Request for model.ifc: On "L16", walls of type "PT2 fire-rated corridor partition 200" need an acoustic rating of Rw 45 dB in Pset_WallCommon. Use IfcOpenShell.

First a look at what the model holds.

```python
import ifcopenshell
import ifcopenshell.util.element

model = ifcopenshell.open("model.ifc")
print(model.schema)
storey = next(s for s in model.by_type("IfcBuildingStorey") if s.Name == "L16")
walls = [e for e in ifcopenshell.util.element.get_decomposition(storey) if e.is_a("IfcWall")]
seen = {}
for e in walls:
    element_type = ifcopenshell.util.element.get_type(e)
    key = (element_type.Name if element_type != e and element_type else None, ifcopenshell.util.element.get_pset(e, "Pset_WallCommon", "AcousticRating"))
    seen[key] = seen.get(key, 0) + 1
for (name, value), count in sorted(seen.items(), key=str):
    print(count, "x", name, "|", value)
```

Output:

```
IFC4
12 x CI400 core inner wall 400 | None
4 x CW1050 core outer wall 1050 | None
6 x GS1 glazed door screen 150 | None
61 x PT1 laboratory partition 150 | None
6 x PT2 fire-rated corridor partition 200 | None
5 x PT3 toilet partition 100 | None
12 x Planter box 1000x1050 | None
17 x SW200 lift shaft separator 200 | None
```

```python
import ifcopenshell
import ifcopenshell.api.pset
import ifcopenshell.util.element

model = ifcopenshell.open("model.ifc")

storey = next(s for s in model.by_type("IfcBuildingStorey") if s.Name == "L16")
walls = [e for e in ifcopenshell.util.element.get_decomposition(storey) if e.is_a("IfcWall")]

count = 0
for e in walls:
    element_type = ifcopenshell.util.element.get_type(e)
    if element_type in (None, e) or element_type.Name != "PT2 fire-rated corridor partition 200":
        continue
    found = ifcopenshell.util.element.get_pset(e, "Pset_WallCommon", should_inherit=False)
    if found:
        pset = model.by_id(found["id"])
        if len(ifcopenshell.util.element.get_elements_by_pset(pset)) > 1:
            pset = ifcopenshell.api.pset.unshare_pset(model, products=[e], pset=pset)[0]
    else:
        pset = ifcopenshell.api.pset.add_pset(model, product=e, name="Pset_WallCommon")
    ifcopenshell.api.pset.edit_pset(model, pset=pset, properties={"AcousticRating": "Rw 45 dB"})
    count += 1

print(count, "walls updated")

model.write("model_edited.ifc")
```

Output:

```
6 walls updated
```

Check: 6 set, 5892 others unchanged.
